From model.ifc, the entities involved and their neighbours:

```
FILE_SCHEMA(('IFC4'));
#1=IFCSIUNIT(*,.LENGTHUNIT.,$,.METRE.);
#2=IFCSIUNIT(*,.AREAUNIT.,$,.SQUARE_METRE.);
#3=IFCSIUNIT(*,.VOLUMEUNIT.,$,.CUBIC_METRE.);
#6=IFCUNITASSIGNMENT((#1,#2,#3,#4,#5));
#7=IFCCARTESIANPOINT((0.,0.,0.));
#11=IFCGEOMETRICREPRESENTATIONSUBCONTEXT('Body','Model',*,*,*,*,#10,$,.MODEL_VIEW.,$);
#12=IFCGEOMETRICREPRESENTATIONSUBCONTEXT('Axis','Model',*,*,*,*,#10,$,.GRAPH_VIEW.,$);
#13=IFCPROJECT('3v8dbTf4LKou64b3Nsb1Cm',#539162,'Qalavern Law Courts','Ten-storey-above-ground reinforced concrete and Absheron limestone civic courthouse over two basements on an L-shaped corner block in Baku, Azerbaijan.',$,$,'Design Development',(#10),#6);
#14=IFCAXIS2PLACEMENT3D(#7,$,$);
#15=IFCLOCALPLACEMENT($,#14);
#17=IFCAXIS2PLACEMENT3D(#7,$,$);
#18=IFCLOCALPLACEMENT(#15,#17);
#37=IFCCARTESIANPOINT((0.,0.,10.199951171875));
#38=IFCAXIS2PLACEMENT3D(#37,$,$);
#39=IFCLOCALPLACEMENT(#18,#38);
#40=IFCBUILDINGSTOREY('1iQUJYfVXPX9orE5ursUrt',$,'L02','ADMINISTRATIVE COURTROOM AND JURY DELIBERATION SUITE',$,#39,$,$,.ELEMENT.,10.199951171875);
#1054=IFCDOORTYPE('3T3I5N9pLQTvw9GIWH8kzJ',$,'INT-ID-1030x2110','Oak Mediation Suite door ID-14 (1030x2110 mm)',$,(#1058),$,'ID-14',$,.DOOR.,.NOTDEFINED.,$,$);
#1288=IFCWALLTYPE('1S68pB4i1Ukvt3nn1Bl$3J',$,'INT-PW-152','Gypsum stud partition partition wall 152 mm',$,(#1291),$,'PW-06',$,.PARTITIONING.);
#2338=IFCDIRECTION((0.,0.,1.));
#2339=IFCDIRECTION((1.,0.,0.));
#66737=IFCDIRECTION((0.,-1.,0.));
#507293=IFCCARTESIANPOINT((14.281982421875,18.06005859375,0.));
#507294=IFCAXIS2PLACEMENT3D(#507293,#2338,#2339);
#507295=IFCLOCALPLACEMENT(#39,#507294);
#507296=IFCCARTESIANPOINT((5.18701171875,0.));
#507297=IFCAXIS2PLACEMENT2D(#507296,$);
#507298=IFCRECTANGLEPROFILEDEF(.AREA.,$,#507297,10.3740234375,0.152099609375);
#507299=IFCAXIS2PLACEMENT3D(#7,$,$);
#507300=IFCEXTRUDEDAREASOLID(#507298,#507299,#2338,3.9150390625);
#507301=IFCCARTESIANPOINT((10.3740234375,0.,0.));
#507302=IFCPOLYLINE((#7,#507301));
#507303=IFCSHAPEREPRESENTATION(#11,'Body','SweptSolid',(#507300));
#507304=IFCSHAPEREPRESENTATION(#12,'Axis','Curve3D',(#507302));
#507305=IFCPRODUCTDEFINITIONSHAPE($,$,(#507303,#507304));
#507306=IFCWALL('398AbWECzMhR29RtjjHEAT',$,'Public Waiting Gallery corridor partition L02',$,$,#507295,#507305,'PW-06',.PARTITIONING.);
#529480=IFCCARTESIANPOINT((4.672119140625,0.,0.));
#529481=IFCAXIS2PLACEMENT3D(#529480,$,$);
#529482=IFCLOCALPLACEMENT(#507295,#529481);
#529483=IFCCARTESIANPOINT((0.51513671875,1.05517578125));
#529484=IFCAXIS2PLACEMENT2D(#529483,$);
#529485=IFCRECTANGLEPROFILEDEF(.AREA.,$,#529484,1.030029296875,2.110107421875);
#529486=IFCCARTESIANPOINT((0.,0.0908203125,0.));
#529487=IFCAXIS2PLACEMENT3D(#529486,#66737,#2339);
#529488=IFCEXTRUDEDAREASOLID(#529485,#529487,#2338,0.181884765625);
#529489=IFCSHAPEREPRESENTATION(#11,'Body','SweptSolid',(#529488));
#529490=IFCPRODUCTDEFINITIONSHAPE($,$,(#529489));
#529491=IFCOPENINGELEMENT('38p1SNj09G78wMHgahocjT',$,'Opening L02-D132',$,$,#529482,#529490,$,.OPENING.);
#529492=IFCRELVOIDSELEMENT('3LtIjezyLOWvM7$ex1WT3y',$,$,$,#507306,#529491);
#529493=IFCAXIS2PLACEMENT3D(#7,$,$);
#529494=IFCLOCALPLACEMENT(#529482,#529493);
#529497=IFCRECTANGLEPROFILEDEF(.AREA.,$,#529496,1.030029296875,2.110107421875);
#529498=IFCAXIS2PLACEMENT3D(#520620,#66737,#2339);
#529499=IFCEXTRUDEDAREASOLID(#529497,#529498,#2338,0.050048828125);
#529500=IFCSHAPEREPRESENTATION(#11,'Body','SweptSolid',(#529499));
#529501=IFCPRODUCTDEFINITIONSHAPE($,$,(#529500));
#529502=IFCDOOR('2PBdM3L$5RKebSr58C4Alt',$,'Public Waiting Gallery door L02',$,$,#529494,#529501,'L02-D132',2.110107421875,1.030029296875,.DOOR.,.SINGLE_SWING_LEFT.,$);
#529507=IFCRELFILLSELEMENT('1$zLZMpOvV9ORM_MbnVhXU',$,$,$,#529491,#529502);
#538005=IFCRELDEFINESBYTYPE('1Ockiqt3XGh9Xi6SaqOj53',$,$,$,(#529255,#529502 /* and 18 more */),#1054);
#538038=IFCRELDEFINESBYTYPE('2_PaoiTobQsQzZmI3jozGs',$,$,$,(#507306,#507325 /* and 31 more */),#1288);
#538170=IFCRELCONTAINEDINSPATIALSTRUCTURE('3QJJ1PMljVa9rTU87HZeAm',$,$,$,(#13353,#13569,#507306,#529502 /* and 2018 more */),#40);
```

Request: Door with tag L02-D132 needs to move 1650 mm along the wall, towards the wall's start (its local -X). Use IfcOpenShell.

```python
import ifcopenshell
import ifcopenshell.api.geometry
import ifcopenshell.util.placement
import ifcopenshell.util.unit

model = ifcopenshell.open("model.ifc")
unit_scale = ifcopenshell.util.unit.calculate_unit_scale(model)

door = model.by_guid("2PBdM3L$5RKebSr58C4Alt")
opening = door.FillsVoids[0].RelatingOpeningElement
wall = opening.VoidsElements[0].RelatingBuildingElement

wall_matrix = ifcopenshell.util.placement.get_local_placement(wall.ObjectPlacement)
shift = wall_matrix[:3, 0] * -1.65 / unit_scale
before = ifcopenshell.util.placement.get_local_placement(door.ObjectPlacement)[:3, 3].copy()

# The door is placed relative to its opening, so it follows when the opening moves.
matrix = ifcopenshell.util.placement.get_local_placement(opening.ObjectPlacement)
matrix[:3, 3] += shift
ifcopenshell.api.geometry.edit_object_placement(
    model, product=opening, matrix=matrix, is_si=False, should_transform_children=True
)

after = ifcopenshell.util.placement.get_local_placement(door.ObjectPlacement)[:3, 3]
print("door moved by", (after - before).round(3) + 0.0)

model.write("model_updated.ifc")
```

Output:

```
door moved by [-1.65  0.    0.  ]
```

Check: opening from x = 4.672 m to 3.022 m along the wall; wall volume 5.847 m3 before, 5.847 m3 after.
